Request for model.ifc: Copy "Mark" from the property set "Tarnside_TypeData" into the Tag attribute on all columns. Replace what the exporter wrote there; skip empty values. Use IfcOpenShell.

First a look at what the model holds.

```python
import ifcopenshell
import ifcopenshell.util.element

model = ifcopenshell.open("model.ifc")
print(model.schema)
columns = model.by_type("IfcColumn")
print(len(columns), "columns")
for e in columns[:8]:
    source = ifcopenshell.util.element.get_pset(e, "Tarnside_TypeData", "Mark")
    target = e.Tag
    print(e.id(), repr(source), repr(target), sep=" | ")
```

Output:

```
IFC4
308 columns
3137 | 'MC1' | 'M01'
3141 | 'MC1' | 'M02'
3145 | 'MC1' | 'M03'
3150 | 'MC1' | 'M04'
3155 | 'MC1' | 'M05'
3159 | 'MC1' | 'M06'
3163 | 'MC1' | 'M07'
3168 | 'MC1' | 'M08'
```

```python
import ifcopenshell
import ifcopenshell.util.element

model = ifcopenshell.open("model.ifc")

count = 0
for e in model.by_type("IfcColumn"):
    value = ifcopenshell.util.element.get_pset(e, "Tarnside_TypeData", "Mark")
    current = e.Tag
    if not value or not value.strip() or current == value:
        continue
    e.Tag = value
    count += 1

print(count, "columns updated")

model.write("model_v2.ifc")
```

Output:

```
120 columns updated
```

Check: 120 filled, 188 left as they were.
